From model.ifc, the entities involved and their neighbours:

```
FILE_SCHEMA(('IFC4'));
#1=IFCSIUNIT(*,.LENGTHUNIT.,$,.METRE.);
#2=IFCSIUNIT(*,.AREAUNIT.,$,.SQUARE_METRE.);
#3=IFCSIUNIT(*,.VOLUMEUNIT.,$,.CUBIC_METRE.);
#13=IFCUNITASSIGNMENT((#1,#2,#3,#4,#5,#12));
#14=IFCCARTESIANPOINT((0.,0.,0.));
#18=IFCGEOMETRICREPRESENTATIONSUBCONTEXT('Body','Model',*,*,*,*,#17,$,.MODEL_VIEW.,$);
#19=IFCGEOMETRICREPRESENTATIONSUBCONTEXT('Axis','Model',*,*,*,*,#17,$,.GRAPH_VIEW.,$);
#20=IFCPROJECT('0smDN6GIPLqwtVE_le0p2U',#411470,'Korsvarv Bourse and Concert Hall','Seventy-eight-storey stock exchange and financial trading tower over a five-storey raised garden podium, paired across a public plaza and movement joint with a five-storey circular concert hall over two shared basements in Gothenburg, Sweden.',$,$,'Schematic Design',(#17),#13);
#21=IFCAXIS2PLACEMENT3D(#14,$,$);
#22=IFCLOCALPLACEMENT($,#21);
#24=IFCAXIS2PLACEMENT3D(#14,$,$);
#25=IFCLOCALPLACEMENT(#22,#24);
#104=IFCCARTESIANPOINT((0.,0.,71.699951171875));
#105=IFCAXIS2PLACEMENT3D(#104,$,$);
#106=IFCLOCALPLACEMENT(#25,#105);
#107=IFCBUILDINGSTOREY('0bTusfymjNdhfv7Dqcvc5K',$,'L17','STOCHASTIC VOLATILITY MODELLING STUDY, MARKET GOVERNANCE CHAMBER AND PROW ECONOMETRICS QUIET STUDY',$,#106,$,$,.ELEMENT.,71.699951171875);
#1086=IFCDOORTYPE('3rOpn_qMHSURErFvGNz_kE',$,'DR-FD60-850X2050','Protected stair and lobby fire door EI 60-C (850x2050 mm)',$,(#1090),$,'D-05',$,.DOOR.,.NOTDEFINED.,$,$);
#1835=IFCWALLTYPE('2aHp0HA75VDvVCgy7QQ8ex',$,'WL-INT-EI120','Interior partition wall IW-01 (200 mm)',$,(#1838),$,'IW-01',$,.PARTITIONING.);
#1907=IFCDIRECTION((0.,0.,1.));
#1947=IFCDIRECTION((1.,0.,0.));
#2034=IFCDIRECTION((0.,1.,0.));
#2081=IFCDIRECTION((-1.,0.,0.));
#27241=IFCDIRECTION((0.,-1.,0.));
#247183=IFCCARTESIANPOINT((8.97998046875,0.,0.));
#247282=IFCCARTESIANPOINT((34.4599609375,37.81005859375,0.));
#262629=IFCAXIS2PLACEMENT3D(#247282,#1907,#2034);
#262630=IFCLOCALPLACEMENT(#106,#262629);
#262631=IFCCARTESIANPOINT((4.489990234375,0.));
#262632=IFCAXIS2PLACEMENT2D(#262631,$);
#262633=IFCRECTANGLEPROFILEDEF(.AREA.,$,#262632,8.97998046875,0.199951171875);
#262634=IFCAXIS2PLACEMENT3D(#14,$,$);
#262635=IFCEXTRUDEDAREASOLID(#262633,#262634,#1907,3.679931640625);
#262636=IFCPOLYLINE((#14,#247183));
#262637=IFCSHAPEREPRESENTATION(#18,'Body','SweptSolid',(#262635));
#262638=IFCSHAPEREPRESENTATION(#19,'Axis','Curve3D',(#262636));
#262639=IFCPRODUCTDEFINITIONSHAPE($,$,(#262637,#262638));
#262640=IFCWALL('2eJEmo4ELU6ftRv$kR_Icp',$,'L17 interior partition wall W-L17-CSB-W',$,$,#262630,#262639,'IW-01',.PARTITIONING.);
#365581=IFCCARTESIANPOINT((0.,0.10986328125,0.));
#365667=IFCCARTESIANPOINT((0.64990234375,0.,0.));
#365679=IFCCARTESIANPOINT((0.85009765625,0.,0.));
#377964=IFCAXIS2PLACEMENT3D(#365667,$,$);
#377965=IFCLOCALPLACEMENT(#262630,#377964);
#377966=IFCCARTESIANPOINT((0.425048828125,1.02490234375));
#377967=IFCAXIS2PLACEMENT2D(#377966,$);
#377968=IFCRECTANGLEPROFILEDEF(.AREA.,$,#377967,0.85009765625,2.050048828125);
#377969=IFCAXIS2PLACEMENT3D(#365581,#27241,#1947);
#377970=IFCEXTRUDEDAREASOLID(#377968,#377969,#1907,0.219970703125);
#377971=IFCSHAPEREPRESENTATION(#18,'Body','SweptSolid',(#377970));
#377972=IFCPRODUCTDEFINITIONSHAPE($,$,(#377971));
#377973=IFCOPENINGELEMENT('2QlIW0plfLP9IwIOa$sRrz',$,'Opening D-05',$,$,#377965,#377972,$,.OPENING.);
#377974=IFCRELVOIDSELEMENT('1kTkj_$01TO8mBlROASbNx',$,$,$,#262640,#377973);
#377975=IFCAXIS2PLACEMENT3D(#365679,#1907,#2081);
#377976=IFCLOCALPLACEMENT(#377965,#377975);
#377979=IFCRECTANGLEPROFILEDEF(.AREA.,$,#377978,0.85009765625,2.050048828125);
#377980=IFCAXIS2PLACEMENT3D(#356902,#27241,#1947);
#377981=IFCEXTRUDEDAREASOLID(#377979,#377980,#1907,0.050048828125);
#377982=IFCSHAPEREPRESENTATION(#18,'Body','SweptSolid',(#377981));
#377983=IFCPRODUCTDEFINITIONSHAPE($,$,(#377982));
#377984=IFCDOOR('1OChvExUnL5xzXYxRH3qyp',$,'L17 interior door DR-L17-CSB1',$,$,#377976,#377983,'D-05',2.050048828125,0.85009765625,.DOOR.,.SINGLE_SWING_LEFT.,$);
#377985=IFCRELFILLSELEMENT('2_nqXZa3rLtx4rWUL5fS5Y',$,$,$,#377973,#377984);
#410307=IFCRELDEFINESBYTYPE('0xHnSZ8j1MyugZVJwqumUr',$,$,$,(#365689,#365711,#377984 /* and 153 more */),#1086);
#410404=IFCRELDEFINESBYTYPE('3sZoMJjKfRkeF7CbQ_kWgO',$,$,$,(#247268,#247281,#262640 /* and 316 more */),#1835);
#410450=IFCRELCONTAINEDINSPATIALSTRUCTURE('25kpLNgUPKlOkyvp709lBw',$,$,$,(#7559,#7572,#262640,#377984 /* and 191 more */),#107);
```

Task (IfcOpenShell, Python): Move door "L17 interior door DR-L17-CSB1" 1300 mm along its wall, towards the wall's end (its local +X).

```python
import ifcopenshell
import ifcopenshell.api.geometry
import ifcopenshell.util.placement
import ifcopenshell.util.unit

model = ifcopenshell.open("model.ifc")
unit_scale = ifcopenshell.util.unit.calculate_unit_scale(model)

door = model.by_guid("1OChvExUnL5xzXYxRH3qyp")
opening = door.FillsVoids[0].RelatingOpeningElement
wall = opening.VoidsElements[0].RelatingBuildingElement

wall_matrix = ifcopenshell.util.placement.get_local_placement(wall.ObjectPlacement)
shift = wall_matrix[:3, 0] * 1.3 / unit_scale
before = ifcopenshell.util.placement.get_local_placement(door.ObjectPlacement)[:3, 3].copy()

# The door is placed relative to its opening, so it follows when the opening moves.
matrix = ifcopenshell.util.placement.get_local_placement(opening.ObjectPlacement)
matrix[:3, 3] += shift
ifcopenshell.api.geometry.edit_object_placement(
    model, product=opening, matrix=matrix, is_si=False, should_transform_children=True
)

after = ifcopenshell.util.placement.get_local_placement(door.ObjectPlacement)[:3, 3]
print("door moved by", (after - before).round(3) + 0.0)

model.write("model_v2.ifc")
```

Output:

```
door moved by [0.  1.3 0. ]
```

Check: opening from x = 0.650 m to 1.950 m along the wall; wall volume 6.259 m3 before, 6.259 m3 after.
